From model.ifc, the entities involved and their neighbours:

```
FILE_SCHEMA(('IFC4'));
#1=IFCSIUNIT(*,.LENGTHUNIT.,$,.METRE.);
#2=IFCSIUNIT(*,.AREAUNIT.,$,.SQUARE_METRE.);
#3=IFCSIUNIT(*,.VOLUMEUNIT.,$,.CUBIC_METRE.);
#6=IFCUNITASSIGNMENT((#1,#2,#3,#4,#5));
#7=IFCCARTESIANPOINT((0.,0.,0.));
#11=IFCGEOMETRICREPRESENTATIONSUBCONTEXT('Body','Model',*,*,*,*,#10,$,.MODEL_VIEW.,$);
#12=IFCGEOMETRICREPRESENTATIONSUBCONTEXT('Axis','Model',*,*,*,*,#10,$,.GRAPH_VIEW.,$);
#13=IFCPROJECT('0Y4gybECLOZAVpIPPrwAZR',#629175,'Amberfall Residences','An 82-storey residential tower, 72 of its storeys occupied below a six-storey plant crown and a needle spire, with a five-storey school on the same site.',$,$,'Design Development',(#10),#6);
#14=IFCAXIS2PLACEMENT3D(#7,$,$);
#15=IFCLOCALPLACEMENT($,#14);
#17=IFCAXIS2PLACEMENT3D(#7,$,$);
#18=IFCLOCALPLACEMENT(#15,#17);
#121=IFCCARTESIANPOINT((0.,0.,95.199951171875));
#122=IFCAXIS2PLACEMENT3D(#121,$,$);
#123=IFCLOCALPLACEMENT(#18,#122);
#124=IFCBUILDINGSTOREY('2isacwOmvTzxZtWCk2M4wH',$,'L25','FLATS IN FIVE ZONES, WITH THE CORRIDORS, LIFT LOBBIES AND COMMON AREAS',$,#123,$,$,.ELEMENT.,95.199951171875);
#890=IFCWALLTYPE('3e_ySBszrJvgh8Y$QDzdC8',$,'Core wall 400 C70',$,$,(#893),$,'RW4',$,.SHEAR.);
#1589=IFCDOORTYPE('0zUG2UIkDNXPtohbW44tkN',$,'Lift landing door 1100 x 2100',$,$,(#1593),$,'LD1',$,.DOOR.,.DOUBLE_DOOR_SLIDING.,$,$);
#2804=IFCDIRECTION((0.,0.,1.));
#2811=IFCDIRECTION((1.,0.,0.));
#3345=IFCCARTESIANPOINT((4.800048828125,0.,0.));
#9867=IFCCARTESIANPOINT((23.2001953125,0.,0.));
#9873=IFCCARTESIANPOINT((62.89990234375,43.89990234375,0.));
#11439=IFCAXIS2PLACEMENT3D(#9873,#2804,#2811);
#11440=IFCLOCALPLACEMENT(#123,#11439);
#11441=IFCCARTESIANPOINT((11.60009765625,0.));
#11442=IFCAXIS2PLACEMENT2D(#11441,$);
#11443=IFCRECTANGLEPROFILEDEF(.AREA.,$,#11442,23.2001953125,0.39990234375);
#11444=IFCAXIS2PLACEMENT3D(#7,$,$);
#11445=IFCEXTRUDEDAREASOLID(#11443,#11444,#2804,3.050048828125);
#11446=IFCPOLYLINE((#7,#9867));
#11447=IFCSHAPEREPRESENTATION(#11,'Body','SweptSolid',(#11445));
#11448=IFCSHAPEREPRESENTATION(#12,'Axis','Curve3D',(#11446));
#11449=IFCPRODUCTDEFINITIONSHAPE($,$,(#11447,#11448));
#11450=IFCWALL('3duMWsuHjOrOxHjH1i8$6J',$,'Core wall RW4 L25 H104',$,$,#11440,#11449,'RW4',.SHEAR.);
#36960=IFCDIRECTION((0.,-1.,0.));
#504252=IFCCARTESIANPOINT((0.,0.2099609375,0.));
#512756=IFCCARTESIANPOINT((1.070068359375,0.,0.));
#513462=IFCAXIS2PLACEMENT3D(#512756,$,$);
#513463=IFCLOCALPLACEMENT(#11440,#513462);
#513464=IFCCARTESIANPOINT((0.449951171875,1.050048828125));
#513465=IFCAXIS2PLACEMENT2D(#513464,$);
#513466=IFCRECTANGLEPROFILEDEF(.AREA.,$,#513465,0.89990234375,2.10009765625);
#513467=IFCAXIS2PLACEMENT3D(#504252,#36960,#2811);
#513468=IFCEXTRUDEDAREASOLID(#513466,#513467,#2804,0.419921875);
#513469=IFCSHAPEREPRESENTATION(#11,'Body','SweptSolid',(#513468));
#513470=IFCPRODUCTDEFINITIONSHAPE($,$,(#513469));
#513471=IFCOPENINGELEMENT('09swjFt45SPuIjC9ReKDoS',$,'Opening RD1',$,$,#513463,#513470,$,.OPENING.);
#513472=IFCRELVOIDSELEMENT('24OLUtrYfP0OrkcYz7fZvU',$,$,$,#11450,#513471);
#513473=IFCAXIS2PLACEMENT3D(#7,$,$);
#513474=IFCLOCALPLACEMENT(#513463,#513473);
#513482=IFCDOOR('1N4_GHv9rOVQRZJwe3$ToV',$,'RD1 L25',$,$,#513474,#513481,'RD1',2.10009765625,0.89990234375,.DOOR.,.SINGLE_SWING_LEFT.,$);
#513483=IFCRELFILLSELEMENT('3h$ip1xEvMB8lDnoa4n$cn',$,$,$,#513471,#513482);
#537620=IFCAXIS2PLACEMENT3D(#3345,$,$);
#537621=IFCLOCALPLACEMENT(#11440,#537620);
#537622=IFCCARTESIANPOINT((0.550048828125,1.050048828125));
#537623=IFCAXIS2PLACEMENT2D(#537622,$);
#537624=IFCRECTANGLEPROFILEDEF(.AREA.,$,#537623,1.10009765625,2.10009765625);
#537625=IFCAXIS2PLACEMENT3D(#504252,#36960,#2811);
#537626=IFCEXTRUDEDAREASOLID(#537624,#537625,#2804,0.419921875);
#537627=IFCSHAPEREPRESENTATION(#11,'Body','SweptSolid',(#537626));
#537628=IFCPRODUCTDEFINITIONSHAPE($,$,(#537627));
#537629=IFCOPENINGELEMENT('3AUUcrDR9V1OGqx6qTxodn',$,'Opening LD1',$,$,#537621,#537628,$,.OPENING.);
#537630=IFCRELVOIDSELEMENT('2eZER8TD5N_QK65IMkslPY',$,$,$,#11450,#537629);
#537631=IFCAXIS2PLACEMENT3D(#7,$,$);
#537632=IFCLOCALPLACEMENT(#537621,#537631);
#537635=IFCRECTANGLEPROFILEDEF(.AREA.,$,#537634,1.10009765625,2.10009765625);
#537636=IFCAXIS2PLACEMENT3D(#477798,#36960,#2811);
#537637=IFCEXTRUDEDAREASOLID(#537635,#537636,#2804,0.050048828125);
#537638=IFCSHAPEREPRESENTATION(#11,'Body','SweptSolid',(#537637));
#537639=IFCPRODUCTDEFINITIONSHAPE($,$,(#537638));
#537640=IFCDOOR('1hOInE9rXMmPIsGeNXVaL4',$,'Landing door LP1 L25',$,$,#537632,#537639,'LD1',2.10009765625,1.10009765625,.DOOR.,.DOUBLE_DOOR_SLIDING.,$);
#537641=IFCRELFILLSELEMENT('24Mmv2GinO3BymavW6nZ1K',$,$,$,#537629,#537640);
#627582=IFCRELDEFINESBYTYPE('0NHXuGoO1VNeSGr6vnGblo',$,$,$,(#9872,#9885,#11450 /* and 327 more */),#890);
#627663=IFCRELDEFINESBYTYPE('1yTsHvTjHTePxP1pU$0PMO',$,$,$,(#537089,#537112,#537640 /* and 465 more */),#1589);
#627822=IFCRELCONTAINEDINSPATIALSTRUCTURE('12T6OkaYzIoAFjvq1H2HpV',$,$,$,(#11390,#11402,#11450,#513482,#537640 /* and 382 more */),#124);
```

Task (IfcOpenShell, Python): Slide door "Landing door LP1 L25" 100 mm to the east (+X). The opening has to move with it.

```python
import ifcopenshell
import ifcopenshell.api.geometry
import ifcopenshell.util.placement

model = ifcopenshell.open("model.ifc")

door = model.by_guid("1hOInE9rXMmPIsGeNXVaL4")
opening = door.FillsVoids[0].RelatingOpeningElement
wall = opening.VoidsElements[0].RelatingBuildingElement

wall_matrix = ifcopenshell.util.placement.get_local_placement(wall.ObjectPlacement)
shift = wall_matrix[:3, 0] * 0.1
before = ifcopenshell.util.placement.get_local_placement(door.ObjectPlacement)[:3, 3].copy()

# The door is placed relative to its opening, so it follows when the opening moves.
matrix = ifcopenshell.util.placement.get_local_placement(opening.ObjectPlacement)
matrix[:3, 3] += shift
ifcopenshell.api.geometry.edit_object_placement(
    model, product=opening, matrix=matrix, is_si=False, should_transform_children=True
)

after = ifcopenshell.util.placement.get_local_placement(door.ObjectPlacement)[:3, 3]
print("door moved by", (after - before).round(3) + 0.0)

model.write("model-out.ifc")
```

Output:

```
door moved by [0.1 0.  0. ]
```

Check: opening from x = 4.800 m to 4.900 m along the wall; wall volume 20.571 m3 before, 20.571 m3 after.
